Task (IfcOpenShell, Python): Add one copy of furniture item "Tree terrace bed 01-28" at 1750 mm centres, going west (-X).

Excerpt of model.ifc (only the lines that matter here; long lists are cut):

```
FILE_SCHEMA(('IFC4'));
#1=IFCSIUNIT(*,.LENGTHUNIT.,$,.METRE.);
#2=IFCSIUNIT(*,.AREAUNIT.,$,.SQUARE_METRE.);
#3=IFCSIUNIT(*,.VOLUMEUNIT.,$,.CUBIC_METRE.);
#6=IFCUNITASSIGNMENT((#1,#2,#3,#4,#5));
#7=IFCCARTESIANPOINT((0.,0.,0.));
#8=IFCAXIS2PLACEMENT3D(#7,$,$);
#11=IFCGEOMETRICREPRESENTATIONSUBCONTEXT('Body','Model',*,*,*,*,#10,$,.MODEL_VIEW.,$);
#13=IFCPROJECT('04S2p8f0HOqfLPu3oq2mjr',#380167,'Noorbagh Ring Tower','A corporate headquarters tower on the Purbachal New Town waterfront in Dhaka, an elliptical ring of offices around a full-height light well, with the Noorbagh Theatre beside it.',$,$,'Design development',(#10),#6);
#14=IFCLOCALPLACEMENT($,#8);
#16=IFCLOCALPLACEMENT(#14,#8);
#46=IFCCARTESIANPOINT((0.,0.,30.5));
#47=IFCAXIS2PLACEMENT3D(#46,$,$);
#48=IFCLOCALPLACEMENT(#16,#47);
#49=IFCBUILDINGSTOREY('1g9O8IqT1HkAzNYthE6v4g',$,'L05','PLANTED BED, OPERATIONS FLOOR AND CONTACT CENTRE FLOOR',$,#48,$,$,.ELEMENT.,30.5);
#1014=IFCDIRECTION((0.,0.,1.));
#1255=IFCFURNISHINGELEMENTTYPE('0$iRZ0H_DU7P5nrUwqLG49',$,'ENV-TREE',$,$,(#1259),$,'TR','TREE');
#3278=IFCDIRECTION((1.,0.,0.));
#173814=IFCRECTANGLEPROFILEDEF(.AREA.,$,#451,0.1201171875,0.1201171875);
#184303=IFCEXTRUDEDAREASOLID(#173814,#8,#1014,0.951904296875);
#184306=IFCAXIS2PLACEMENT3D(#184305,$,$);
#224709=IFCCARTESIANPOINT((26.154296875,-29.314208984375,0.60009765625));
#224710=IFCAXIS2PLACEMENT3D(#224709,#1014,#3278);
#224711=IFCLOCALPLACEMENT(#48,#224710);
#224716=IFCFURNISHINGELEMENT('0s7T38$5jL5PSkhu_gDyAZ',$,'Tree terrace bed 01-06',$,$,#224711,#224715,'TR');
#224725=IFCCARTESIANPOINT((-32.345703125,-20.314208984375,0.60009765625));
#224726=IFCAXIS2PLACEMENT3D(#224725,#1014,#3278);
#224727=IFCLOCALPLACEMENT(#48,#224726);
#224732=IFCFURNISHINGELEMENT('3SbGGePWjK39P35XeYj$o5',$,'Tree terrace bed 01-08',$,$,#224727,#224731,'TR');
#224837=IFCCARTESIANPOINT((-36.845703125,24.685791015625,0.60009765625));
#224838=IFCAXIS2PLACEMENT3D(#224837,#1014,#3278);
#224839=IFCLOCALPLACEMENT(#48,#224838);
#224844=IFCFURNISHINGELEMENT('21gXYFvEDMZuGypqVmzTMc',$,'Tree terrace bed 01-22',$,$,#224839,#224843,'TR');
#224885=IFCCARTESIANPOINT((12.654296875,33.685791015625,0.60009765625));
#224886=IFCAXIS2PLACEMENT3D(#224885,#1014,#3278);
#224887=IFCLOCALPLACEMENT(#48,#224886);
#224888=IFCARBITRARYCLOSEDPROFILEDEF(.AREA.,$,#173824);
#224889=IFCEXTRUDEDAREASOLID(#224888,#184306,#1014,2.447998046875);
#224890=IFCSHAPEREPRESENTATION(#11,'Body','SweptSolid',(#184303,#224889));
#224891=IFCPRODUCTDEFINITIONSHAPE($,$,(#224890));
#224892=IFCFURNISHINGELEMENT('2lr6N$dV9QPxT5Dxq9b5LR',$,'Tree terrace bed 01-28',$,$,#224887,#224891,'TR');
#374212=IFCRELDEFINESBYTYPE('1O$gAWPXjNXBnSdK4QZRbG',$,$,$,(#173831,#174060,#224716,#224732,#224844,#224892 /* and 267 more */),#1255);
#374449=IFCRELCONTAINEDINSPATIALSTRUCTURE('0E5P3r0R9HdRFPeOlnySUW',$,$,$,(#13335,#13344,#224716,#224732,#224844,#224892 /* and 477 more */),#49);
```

```python
import numpy as np
import ifcopenshell
import ifcopenshell.api.geometry
import ifcopenshell.api.root
import ifcopenshell.util.element
import ifcopenshell.util.placement
import ifcopenshell.util.unit

model = ifcopenshell.open("model.ifc")
unit_scale = ifcopenshell.util.unit.calculate_unit_scale(model)

source = model.by_guid("2lr6N$dV9QPxT5Dxq9b5LR")
base = ifcopenshell.util.placement.get_local_placement(source.ObjectPlacement)
step = np.array([-1.0, 0.0, 0.0]) * 1.75 / unit_scale

for i in range(1, 2):
    copy = ifcopenshell.api.root.copy_class(model, product=source)
    copy.Representation = ifcopenshell.util.element.copy_deep(
        model, source.Representation, exclude=["IfcGeometricRepresentationContext", "IfcRepresentationMap"]
    )
    copy.Tag = None
    matrix = base.copy()
    matrix[:3, 3] += i * step
    print("added at", matrix[:3, 3].round(3) + 0.0)
    ifcopenshell.api.geometry.edit_object_placement(model, product=copy, matrix=matrix, is_si=False)

model.write("model_v2.ifc")
```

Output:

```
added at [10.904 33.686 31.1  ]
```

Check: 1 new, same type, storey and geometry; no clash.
